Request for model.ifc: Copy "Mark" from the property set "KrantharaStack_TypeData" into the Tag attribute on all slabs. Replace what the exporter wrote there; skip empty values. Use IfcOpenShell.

First a look at what the model holds.

```python
import ifcopenshell
import ifcopenshell.util.element

model = ifcopenshell.open("model.ifc")
print(model.schema)
slabs = model.by_type("IfcSlab")
print(len(slabs), "slabs")
for e in slabs[:8]:
    source = ifcopenshell.util.element.get_pset(e, "KrantharaStack_TypeData", "Mark")
    target = e.Tag
    print(e.id(), repr(source), repr(target), sep=" | ")
```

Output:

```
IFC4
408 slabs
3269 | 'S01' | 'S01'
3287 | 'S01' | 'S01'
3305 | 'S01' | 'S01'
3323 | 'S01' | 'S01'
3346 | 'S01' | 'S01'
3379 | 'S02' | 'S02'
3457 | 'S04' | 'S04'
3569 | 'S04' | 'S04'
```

```python
import ifcopenshell
import ifcopenshell.util.element

model = ifcopenshell.open("model.ifc")

count = 0
for e in model.by_type("IfcSlab"):
    value = ifcopenshell.util.element.get_pset(e, "KrantharaStack_TypeData", "Mark")
    current = e.Tag
    if not value or not value.strip() or current == value:
        continue
    e.Tag = value
    count += 1

print(count, "slabs updated")

model.write("model_v2.ifc")
```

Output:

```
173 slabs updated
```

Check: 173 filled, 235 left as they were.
